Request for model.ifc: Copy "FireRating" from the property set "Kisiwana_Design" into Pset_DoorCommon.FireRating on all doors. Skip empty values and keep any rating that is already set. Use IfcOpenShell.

First a look at what the model holds.

```python
import ifcopenshell
import ifcopenshell.util.element

model = ifcopenshell.open("model.ifc")
print(model.schema)
doors = model.by_type("IfcDoor")
print(len(doors), "doors")
for e in doors[:8]:
    source = ifcopenshell.util.element.get_pset(e, "Kisiwana_Design", "FireRating")
    target = ifcopenshell.util.element.get_pset(e, "Pset_DoorCommon", "FireRating")
    print(e.id(), repr(source), repr(target), sep=" | ")
```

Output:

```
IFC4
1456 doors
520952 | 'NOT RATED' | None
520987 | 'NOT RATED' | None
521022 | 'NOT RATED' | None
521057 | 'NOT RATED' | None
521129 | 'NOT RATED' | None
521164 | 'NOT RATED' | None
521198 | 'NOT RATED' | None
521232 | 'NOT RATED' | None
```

```python
import ifcopenshell
import ifcopenshell.api.pset
import ifcopenshell.util.element

model = ifcopenshell.open("model.ifc")

count = 0
for e in model.by_type("IfcDoor"):
    value = ifcopenshell.util.element.get_pset(e, "Kisiwana_Design", "FireRating")
    current = ifcopenshell.util.element.get_pset(e, "Pset_DoorCommon", "FireRating")
    if not value or not value.strip() or current:
        continue
    # add_pset returns the element's existing set when there is one.
    pset = ifcopenshell.api.pset.add_pset(model, product=e, name="Pset_DoorCommon")
    ifcopenshell.api.pset.edit_pset(model, pset=pset, properties={"FireRating": value})
    count += 1

print(count, "doors updated")

model.write("model-out.ifc")
```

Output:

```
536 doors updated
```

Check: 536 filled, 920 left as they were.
